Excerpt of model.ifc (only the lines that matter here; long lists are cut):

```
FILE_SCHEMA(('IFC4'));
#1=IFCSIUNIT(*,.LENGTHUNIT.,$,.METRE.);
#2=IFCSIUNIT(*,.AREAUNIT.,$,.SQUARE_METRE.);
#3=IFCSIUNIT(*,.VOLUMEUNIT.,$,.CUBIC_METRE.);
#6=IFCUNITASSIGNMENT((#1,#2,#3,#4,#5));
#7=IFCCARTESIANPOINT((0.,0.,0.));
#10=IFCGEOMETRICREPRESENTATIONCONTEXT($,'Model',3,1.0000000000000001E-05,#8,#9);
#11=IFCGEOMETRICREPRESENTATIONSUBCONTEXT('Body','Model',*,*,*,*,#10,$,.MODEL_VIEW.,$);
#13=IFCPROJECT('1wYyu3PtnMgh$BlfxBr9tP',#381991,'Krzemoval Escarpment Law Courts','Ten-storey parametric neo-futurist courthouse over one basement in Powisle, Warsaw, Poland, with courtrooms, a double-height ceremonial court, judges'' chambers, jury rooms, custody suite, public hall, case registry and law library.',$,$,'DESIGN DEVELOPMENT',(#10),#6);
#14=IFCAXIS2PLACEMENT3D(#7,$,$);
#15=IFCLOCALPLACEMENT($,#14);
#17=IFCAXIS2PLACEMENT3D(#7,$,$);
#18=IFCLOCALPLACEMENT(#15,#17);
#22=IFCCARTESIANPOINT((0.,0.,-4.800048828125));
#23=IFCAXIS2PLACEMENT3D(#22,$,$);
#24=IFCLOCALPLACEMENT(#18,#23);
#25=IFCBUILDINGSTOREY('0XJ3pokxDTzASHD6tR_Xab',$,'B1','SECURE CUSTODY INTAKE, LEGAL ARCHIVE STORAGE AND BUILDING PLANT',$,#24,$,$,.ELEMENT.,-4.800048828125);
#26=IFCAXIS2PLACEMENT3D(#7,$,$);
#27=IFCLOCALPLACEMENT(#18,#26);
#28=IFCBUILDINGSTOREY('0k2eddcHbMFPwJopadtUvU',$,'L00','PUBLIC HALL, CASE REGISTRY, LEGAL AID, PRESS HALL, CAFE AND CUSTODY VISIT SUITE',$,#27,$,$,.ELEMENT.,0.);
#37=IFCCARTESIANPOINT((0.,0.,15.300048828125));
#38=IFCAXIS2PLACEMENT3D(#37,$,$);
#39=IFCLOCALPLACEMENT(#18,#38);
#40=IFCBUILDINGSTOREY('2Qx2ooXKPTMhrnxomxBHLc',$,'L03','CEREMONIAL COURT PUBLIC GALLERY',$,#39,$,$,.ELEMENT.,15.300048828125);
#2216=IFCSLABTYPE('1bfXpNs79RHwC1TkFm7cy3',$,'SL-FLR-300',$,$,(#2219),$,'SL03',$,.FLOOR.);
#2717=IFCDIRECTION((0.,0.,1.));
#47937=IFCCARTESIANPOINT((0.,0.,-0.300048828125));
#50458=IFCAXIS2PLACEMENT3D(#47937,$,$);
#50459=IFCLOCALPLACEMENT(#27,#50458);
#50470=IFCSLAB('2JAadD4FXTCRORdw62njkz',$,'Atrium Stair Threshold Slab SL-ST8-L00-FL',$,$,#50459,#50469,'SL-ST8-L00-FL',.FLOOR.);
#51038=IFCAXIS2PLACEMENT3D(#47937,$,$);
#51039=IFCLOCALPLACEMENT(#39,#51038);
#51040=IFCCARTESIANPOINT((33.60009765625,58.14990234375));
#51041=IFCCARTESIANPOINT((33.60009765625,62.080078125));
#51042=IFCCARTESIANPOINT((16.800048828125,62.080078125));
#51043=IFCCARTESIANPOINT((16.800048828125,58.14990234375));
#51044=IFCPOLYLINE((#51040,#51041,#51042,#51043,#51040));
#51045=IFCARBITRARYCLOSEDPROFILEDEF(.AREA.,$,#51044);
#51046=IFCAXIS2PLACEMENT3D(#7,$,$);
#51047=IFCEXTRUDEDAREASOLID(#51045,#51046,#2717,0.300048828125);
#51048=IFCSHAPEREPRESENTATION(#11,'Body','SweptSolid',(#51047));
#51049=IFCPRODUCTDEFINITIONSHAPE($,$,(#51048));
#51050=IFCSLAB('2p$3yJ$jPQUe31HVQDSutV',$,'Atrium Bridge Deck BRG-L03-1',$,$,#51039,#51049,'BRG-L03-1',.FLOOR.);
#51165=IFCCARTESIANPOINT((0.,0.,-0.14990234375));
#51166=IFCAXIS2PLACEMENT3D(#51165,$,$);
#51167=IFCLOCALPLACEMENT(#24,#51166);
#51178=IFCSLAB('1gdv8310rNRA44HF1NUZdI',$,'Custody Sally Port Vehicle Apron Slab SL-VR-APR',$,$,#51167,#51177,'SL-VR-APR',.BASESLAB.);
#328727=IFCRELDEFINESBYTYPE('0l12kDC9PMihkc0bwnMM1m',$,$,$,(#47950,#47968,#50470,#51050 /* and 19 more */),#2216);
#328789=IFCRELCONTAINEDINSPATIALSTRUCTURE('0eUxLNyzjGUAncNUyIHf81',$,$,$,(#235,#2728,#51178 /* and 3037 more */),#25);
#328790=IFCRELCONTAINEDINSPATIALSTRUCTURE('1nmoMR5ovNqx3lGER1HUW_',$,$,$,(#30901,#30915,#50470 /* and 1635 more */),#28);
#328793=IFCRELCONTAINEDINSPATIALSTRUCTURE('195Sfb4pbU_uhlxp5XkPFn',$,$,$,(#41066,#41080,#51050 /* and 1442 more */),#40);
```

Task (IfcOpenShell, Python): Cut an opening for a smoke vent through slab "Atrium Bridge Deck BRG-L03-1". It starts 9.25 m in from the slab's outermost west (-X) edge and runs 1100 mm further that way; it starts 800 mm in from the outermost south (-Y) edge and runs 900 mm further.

```python
import numpy as np
import ifcopenshell
import ifcopenshell.api.feature
import ifcopenshell.api.geometry
import ifcopenshell.api.root
import ifcopenshell.geom
import ifcopenshell.util.placement
import ifcopenshell.util.representation
import ifcopenshell.util.shape
import ifcopenshell.util.unit

model = ifcopenshell.open("model.ifc")
unit_scale = ifcopenshell.util.unit.calculate_unit_scale(model)
settings = ifcopenshell.geom.settings()


def volume(element):
    """Net volume in cubic metres, openings subtracted."""
    shape = ifcopenshell.geom.create_shape(settings, element)
    return ifcopenshell.util.shape.get_volume(shape.geometry)


slab = model.by_id(51050)
before = volume(slab)

# Extent in the slab's own axes, in metres. The edges named are its -X and -Y sides.
slab_shape = ifcopenshell.geom.create_shape(settings, slab)
vertices = ifcopenshell.util.shape.get_vertices(slab_shape.geometry)
x_min, y_min, bottom = vertices.min(axis=0)
top = vertices[:, 2].max()

opening = ifcopenshell.api.root.create_entity(model, ifc_class="IfcOpeningElement", name="Smoke vent opening", predefined_type="OPENING")
context = ifcopenshell.util.representation.get_context(model, "Model", "Body", "MODEL_VIEW")
width, depth = 1.1, 0.9
outline = [(0.0, 0.0), (width, 0.0), (width, depth), (0.0, depth), (0.0, 0.0)]
# Overshoot both faces by 50 mm so the cut is clean.
shape = ifcopenshell.api.geometry.add_slab_representation(
    model, context=context, depth=top - bottom + 0.1, polyline=outline
)
ifcopenshell.api.geometry.assign_representation(model, product=opening, representation=shape)

matrix = ifcopenshell.util.placement.get_local_placement(slab.ObjectPlacement)
matrix[:, 3] = matrix @ np.append(np.array([x_min + 9.25, y_min + 0.8, bottom - 0.05]) / unit_scale, 1.0)
ifcopenshell.api.geometry.edit_object_placement(model, product=opening, matrix=matrix, is_si=False)
ifcopenshell.api.feature.add_feature(model, feature=opening, element=slab)

after = volume(slab)

print(f"slab volume {before:.3f} -> {after:.3f} m3")

model.write("model_rev.ifc")
```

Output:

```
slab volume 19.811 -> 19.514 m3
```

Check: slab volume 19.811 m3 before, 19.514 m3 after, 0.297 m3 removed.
